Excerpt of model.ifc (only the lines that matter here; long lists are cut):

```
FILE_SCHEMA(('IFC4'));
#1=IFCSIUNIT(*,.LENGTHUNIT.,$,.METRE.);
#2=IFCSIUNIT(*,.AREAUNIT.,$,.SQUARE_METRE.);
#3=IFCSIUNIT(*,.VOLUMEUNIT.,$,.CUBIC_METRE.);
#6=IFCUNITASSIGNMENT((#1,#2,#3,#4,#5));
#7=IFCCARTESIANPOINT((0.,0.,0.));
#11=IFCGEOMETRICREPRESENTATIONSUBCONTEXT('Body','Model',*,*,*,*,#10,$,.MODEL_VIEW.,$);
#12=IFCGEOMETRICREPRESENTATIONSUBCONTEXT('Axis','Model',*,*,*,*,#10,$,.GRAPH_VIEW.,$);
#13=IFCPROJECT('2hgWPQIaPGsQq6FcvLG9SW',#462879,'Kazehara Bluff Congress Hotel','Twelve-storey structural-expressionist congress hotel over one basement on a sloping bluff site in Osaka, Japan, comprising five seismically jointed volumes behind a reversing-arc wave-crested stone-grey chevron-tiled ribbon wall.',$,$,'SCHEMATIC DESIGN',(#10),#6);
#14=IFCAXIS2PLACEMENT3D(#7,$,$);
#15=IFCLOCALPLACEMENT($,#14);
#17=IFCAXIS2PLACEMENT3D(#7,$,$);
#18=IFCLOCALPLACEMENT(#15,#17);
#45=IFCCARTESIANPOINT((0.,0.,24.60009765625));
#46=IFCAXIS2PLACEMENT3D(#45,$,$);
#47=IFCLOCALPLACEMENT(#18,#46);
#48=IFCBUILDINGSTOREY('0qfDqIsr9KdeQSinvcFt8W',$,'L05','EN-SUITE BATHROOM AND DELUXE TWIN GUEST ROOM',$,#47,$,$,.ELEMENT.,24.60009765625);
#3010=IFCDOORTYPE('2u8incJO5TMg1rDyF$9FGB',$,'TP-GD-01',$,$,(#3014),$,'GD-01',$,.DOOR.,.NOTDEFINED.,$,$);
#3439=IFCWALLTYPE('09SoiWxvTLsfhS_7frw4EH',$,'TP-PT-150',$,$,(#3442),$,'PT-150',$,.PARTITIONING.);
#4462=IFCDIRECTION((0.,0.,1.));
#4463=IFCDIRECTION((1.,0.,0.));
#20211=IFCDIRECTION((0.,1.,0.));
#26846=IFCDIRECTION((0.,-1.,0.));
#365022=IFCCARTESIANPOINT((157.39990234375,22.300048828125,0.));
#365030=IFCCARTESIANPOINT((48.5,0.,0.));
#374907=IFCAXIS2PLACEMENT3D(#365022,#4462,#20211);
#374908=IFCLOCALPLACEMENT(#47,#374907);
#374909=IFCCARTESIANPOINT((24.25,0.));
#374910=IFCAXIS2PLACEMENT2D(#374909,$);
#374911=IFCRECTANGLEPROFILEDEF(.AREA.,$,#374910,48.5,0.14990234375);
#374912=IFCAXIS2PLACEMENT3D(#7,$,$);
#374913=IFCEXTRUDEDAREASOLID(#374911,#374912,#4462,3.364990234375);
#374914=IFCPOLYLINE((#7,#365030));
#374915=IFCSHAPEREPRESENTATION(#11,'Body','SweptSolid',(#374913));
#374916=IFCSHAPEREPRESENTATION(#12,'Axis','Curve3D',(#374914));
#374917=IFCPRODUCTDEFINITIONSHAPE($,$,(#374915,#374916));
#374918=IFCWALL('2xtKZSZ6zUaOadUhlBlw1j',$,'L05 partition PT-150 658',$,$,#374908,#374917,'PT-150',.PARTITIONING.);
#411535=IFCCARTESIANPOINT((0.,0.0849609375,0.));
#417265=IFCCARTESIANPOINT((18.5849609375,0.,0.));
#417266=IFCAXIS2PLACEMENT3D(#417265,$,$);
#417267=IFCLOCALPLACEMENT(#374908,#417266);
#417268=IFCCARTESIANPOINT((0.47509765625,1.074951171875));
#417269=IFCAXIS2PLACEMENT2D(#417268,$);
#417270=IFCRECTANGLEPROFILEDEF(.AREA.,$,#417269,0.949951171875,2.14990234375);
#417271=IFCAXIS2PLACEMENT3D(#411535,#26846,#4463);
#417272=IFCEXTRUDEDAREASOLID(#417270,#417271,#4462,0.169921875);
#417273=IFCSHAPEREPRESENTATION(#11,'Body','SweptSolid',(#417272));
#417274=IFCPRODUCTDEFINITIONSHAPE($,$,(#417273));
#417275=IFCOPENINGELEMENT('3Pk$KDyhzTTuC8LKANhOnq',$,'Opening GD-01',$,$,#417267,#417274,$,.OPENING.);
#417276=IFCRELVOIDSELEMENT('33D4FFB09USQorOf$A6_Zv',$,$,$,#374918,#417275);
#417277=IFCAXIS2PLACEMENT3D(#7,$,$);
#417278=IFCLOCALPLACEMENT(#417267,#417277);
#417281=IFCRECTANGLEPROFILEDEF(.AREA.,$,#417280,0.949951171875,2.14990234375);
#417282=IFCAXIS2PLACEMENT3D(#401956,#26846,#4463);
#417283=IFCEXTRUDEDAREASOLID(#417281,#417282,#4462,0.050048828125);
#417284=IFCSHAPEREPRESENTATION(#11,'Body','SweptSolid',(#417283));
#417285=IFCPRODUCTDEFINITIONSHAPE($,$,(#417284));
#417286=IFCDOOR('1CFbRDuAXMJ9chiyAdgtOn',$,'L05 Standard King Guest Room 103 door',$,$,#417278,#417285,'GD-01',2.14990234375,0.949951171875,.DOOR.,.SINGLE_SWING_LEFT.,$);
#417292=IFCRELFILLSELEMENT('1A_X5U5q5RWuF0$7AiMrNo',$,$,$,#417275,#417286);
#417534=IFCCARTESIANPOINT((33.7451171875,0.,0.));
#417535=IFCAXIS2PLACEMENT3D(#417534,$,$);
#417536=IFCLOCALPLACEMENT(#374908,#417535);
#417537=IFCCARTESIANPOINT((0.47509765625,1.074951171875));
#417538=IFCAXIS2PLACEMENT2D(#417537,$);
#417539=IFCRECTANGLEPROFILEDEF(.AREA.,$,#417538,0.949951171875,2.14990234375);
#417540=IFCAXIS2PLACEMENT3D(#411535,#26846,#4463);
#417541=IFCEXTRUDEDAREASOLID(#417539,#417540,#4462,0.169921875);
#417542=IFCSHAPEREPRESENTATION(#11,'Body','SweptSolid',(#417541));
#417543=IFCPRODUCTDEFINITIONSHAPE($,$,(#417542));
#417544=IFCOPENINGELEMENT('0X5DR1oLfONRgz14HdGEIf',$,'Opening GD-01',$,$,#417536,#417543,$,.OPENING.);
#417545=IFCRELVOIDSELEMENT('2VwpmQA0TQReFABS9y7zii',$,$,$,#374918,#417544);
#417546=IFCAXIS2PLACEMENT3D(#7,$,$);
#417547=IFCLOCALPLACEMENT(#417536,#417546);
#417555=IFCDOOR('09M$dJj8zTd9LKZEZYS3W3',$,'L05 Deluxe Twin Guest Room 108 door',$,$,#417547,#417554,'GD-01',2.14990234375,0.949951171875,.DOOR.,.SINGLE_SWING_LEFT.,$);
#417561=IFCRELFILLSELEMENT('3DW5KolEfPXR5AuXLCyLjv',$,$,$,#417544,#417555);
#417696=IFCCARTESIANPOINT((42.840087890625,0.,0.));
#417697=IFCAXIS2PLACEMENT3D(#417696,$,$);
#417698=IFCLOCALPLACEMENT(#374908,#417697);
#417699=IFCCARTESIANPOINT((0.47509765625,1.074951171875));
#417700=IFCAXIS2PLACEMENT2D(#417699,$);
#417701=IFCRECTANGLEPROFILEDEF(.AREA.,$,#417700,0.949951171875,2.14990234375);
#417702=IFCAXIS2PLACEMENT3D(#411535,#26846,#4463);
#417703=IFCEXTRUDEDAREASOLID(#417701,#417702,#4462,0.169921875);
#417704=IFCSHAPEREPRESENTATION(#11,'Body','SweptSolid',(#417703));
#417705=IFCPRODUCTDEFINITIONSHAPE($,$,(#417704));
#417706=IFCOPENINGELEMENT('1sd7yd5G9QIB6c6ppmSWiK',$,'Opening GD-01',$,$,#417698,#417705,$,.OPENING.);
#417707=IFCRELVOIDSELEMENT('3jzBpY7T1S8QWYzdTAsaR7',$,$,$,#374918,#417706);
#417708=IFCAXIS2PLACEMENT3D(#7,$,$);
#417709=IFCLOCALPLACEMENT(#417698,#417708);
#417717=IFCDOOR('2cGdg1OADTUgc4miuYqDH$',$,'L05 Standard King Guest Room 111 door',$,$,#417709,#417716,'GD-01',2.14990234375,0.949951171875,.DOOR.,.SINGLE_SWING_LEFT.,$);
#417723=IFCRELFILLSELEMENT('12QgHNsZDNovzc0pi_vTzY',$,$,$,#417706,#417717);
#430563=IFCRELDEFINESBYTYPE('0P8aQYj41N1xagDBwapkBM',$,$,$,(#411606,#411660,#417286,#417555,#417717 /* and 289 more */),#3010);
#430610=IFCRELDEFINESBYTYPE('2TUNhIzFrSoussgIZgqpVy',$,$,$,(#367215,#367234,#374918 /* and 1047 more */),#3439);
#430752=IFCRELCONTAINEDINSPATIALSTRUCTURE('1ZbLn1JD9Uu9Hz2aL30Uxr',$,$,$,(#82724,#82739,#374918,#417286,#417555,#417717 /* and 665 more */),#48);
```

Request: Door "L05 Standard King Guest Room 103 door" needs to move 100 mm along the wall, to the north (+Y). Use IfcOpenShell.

```python
import ifcopenshell
import ifcopenshell.api.geometry
import ifcopenshell.util.placement

model = ifcopenshell.open("model.ifc")

door = model.by_id(417286)
opening = door.FillsVoids[0].RelatingOpeningElement
wall = opening.VoidsElements[0].RelatingBuildingElement

wall_matrix = ifcopenshell.util.placement.get_local_placement(wall.ObjectPlacement)
shift = wall_matrix[:3, 0] * 0.1
before = ifcopenshell.util.placement.get_local_placement(door.ObjectPlacement)[:3, 3].copy()

# The door is placed relative to its opening, so it follows when the opening moves.
matrix = ifcopenshell.util.placement.get_local_placement(opening.ObjectPlacement)
matrix[:3, 3] += shift
ifcopenshell.api.geometry.edit_object_placement(
    model, product=opening, matrix=matrix, is_si=False, should_transform_children=True
)

after = ifcopenshell.util.placement.get_local_placement(door.ObjectPlacement)[:3, 3]
print("door moved by", (after - before).round(3) + 0.0)

model.write("model_edited.ifc")
```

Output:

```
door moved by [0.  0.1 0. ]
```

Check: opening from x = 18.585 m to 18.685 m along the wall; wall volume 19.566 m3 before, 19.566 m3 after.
